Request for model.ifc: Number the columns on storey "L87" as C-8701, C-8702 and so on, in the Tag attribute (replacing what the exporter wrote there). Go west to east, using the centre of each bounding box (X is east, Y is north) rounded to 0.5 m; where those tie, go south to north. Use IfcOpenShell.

First a look at what the model holds.

```python
import ifcopenshell
import ifcopenshell.util.element
import ifcopenshell.util.placement

model = ifcopenshell.open("model.ifc")
print(model.schema)
storey = next(s for s in model.by_type("IfcBuildingStorey") if s.Name == "L87")
columns = [e for e in ifcopenshell.util.element.get_decomposition(storey) if e.is_a("IfcColumn")]
for e in sorted(columns, key=lambda e: e.id()):
    origin = ifcopenshell.util.placement.get_local_placement(e.ObjectPlacement)[:3, 3]
    print(e.id(), e.Tag, e.Name, origin.round(2) + 0.0, sep=" | ")
```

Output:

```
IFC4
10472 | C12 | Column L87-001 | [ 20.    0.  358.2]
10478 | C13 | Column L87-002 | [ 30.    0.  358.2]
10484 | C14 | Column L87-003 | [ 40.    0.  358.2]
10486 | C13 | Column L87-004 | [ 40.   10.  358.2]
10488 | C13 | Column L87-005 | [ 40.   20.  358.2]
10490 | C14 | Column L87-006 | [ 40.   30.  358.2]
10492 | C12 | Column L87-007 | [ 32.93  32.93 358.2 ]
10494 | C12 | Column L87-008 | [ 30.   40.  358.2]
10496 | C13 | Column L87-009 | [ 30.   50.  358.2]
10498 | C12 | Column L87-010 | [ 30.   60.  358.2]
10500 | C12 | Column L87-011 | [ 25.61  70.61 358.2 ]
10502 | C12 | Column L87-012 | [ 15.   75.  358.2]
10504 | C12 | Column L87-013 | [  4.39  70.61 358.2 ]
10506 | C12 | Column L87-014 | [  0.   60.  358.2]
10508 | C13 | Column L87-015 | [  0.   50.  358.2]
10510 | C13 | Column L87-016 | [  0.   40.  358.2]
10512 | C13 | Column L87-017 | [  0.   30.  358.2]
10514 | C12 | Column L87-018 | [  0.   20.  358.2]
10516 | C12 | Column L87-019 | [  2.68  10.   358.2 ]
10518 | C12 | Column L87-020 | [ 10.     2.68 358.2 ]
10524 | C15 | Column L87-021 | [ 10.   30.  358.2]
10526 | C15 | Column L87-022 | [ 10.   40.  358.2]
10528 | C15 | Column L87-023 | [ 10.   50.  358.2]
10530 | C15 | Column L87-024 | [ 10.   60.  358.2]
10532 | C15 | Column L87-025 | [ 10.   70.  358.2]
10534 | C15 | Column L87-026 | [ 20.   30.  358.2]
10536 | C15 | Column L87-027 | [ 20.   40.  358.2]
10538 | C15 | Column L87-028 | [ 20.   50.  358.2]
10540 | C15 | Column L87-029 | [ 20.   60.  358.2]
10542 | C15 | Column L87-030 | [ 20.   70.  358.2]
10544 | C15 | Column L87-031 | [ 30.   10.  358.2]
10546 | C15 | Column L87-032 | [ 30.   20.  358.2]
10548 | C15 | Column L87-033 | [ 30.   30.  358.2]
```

```python
import ifcopenshell
import ifcopenshell.geom
import ifcopenshell.util.element
import ifcopenshell.util.shape

model = ifcopenshell.open("model.ifc")
settings = ifcopenshell.geom.settings()
settings.set("use-world-coords", True)


def centre(element):
    shape = ifcopenshell.geom.create_shape(settings, element)
    return ifcopenshell.util.shape.get_bbox_centroid(shape.geometry)


storey = next(s for s in model.by_type("IfcBuildingStorey") if s.Name == "L87")
columns = [e for e in ifcopenshell.util.element.get_decomposition(storey) if e.is_a("IfcColumn")]

# Insertion points can sit at a corner or the storey origin, so sort by the geometry (in metres).
centres = {e: centre(e) for e in columns}
columns.sort(key=lambda e: (round(centres[e][0] / 0.5), centres[e][1]))

for i, e in enumerate(columns, start=1):
    number = f"C-87{i:02d}"
    e.Tag = number
    print(e.id(), number)

model.write("model_edited.ifc")
```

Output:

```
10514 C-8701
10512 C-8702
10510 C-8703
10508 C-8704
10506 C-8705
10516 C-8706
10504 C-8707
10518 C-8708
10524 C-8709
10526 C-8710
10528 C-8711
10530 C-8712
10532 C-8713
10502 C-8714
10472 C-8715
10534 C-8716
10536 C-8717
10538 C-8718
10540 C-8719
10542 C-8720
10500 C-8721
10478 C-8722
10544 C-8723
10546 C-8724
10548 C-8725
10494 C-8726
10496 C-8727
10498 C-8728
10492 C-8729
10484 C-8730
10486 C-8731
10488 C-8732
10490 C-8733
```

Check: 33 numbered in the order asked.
